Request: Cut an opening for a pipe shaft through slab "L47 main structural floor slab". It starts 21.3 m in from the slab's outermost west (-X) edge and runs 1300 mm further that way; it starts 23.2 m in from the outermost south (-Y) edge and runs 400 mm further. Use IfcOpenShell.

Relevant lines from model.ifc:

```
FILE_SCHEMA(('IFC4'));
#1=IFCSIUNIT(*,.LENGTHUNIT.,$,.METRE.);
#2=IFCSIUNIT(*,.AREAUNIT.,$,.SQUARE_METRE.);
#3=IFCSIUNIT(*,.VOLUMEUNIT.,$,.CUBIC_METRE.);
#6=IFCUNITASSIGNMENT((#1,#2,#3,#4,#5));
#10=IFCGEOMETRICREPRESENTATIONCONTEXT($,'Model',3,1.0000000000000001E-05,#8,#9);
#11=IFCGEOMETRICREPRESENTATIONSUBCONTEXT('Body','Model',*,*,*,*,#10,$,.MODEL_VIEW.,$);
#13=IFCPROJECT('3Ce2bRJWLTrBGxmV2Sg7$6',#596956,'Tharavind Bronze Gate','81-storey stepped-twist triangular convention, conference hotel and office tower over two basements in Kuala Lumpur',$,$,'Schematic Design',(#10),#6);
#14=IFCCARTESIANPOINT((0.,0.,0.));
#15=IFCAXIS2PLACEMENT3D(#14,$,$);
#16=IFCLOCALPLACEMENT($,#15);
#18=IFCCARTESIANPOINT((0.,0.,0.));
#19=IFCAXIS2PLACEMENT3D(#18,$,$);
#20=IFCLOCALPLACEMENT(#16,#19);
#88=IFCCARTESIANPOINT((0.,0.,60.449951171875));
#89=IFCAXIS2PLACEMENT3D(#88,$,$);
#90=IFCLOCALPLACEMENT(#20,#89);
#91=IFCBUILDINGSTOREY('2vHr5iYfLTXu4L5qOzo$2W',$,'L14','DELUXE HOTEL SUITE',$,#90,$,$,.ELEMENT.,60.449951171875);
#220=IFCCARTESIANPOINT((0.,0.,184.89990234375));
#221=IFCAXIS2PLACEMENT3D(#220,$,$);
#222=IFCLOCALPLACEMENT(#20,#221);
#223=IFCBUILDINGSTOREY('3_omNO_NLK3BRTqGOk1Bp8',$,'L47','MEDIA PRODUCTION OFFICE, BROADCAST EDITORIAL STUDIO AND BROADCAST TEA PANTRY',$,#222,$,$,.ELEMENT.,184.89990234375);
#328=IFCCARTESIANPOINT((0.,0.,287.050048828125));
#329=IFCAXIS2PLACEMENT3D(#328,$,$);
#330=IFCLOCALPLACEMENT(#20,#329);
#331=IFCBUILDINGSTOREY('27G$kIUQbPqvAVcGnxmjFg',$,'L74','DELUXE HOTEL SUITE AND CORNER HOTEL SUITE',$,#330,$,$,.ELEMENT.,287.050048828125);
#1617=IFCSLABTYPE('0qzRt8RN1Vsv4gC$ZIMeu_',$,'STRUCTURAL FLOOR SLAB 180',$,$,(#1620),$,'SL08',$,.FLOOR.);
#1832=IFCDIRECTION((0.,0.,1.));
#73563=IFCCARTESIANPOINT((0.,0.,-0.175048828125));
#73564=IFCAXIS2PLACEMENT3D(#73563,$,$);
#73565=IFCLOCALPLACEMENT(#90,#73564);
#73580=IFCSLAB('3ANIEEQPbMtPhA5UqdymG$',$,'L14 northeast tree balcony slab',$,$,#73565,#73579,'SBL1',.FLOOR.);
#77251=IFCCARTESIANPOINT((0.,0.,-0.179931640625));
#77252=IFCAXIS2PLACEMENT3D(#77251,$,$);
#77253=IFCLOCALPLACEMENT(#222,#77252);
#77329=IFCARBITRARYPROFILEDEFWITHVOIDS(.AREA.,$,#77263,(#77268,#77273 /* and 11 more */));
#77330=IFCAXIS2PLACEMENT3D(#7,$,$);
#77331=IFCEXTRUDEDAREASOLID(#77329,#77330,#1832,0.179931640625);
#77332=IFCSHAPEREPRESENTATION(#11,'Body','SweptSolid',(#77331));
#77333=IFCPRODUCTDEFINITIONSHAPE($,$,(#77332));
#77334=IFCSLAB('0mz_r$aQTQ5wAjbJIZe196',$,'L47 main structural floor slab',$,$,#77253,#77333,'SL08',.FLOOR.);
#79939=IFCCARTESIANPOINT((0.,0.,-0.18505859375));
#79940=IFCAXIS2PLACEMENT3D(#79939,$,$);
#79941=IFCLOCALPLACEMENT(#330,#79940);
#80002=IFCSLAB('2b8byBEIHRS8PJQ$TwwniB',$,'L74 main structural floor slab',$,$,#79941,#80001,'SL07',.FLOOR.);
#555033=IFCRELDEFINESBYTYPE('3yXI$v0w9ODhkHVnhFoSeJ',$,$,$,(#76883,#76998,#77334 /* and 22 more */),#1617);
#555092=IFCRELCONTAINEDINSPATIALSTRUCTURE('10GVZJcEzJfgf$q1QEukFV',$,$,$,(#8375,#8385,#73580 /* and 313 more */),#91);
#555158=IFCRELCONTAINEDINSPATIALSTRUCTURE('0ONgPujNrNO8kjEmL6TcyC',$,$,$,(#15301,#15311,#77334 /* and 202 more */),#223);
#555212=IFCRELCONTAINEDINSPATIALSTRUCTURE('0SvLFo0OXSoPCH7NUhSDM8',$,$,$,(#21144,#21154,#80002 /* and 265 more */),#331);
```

```python
import numpy as np
import ifcopenshell
import ifcopenshell.api.feature
import ifcopenshell.api.geometry
import ifcopenshell.api.root
import ifcopenshell.geom
import ifcopenshell.util.placement
import ifcopenshell.util.representation
import ifcopenshell.util.shape
import ifcopenshell.util.unit

model = ifcopenshell.open("model.ifc")
unit_scale = ifcopenshell.util.unit.calculate_unit_scale(model)
settings = ifcopenshell.geom.settings()


def volume(element):
    """Net volume in cubic metres, openings subtracted."""
    shape = ifcopenshell.geom.create_shape(settings, element)
    return ifcopenshell.util.shape.get_volume(shape.geometry)


slab = model.by_id(77334)
before = volume(slab)

# Extent in the slab's own axes, in metres. The edges named are its -X and -Y sides.
slab_shape = ifcopenshell.geom.create_shape(settings, slab)
vertices = ifcopenshell.util.shape.get_vertices(slab_shape.geometry)
x_min, y_min, bottom = vertices.min(axis=0)
top = vertices[:, 2].max()

opening = ifcopenshell.api.root.create_entity(model, ifc_class="IfcOpeningElement", name="Pipe shaft opening", predefined_type="OPENING")
context = ifcopenshell.util.representation.get_context(model, "Model", "Body", "MODEL_VIEW")
width, depth = 1.3, 0.4
outline = [(0.0, 0.0), (width, 0.0), (width, depth), (0.0, depth), (0.0, 0.0)]
# Overshoot both faces by 50 mm so the cut is clean.
shape = ifcopenshell.api.geometry.add_slab_representation(
    model, context=context, depth=top - bottom + 0.1, polyline=outline
)
ifcopenshell.api.geometry.assign_representation(model, product=opening, representation=shape)

matrix = ifcopenshell.util.placement.get_local_placement(slab.ObjectPlacement)
matrix[:, 3] = matrix @ np.append(np.array([x_min + 21.3, y_min + 23.2, bottom - 0.05]) / unit_scale, 1.0)
ifcopenshell.api.geometry.edit_object_placement(model, product=opening, matrix=matrix, is_si=False)
ifcopenshell.api.feature.add_feature(model, feature=opening, element=slab)

after = volume(slab)

print(f"slab volume {before:.3f} -> {after:.3f} m3")

model.write("model-out.ifc")
```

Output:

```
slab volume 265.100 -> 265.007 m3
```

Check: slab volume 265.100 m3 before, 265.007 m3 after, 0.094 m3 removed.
